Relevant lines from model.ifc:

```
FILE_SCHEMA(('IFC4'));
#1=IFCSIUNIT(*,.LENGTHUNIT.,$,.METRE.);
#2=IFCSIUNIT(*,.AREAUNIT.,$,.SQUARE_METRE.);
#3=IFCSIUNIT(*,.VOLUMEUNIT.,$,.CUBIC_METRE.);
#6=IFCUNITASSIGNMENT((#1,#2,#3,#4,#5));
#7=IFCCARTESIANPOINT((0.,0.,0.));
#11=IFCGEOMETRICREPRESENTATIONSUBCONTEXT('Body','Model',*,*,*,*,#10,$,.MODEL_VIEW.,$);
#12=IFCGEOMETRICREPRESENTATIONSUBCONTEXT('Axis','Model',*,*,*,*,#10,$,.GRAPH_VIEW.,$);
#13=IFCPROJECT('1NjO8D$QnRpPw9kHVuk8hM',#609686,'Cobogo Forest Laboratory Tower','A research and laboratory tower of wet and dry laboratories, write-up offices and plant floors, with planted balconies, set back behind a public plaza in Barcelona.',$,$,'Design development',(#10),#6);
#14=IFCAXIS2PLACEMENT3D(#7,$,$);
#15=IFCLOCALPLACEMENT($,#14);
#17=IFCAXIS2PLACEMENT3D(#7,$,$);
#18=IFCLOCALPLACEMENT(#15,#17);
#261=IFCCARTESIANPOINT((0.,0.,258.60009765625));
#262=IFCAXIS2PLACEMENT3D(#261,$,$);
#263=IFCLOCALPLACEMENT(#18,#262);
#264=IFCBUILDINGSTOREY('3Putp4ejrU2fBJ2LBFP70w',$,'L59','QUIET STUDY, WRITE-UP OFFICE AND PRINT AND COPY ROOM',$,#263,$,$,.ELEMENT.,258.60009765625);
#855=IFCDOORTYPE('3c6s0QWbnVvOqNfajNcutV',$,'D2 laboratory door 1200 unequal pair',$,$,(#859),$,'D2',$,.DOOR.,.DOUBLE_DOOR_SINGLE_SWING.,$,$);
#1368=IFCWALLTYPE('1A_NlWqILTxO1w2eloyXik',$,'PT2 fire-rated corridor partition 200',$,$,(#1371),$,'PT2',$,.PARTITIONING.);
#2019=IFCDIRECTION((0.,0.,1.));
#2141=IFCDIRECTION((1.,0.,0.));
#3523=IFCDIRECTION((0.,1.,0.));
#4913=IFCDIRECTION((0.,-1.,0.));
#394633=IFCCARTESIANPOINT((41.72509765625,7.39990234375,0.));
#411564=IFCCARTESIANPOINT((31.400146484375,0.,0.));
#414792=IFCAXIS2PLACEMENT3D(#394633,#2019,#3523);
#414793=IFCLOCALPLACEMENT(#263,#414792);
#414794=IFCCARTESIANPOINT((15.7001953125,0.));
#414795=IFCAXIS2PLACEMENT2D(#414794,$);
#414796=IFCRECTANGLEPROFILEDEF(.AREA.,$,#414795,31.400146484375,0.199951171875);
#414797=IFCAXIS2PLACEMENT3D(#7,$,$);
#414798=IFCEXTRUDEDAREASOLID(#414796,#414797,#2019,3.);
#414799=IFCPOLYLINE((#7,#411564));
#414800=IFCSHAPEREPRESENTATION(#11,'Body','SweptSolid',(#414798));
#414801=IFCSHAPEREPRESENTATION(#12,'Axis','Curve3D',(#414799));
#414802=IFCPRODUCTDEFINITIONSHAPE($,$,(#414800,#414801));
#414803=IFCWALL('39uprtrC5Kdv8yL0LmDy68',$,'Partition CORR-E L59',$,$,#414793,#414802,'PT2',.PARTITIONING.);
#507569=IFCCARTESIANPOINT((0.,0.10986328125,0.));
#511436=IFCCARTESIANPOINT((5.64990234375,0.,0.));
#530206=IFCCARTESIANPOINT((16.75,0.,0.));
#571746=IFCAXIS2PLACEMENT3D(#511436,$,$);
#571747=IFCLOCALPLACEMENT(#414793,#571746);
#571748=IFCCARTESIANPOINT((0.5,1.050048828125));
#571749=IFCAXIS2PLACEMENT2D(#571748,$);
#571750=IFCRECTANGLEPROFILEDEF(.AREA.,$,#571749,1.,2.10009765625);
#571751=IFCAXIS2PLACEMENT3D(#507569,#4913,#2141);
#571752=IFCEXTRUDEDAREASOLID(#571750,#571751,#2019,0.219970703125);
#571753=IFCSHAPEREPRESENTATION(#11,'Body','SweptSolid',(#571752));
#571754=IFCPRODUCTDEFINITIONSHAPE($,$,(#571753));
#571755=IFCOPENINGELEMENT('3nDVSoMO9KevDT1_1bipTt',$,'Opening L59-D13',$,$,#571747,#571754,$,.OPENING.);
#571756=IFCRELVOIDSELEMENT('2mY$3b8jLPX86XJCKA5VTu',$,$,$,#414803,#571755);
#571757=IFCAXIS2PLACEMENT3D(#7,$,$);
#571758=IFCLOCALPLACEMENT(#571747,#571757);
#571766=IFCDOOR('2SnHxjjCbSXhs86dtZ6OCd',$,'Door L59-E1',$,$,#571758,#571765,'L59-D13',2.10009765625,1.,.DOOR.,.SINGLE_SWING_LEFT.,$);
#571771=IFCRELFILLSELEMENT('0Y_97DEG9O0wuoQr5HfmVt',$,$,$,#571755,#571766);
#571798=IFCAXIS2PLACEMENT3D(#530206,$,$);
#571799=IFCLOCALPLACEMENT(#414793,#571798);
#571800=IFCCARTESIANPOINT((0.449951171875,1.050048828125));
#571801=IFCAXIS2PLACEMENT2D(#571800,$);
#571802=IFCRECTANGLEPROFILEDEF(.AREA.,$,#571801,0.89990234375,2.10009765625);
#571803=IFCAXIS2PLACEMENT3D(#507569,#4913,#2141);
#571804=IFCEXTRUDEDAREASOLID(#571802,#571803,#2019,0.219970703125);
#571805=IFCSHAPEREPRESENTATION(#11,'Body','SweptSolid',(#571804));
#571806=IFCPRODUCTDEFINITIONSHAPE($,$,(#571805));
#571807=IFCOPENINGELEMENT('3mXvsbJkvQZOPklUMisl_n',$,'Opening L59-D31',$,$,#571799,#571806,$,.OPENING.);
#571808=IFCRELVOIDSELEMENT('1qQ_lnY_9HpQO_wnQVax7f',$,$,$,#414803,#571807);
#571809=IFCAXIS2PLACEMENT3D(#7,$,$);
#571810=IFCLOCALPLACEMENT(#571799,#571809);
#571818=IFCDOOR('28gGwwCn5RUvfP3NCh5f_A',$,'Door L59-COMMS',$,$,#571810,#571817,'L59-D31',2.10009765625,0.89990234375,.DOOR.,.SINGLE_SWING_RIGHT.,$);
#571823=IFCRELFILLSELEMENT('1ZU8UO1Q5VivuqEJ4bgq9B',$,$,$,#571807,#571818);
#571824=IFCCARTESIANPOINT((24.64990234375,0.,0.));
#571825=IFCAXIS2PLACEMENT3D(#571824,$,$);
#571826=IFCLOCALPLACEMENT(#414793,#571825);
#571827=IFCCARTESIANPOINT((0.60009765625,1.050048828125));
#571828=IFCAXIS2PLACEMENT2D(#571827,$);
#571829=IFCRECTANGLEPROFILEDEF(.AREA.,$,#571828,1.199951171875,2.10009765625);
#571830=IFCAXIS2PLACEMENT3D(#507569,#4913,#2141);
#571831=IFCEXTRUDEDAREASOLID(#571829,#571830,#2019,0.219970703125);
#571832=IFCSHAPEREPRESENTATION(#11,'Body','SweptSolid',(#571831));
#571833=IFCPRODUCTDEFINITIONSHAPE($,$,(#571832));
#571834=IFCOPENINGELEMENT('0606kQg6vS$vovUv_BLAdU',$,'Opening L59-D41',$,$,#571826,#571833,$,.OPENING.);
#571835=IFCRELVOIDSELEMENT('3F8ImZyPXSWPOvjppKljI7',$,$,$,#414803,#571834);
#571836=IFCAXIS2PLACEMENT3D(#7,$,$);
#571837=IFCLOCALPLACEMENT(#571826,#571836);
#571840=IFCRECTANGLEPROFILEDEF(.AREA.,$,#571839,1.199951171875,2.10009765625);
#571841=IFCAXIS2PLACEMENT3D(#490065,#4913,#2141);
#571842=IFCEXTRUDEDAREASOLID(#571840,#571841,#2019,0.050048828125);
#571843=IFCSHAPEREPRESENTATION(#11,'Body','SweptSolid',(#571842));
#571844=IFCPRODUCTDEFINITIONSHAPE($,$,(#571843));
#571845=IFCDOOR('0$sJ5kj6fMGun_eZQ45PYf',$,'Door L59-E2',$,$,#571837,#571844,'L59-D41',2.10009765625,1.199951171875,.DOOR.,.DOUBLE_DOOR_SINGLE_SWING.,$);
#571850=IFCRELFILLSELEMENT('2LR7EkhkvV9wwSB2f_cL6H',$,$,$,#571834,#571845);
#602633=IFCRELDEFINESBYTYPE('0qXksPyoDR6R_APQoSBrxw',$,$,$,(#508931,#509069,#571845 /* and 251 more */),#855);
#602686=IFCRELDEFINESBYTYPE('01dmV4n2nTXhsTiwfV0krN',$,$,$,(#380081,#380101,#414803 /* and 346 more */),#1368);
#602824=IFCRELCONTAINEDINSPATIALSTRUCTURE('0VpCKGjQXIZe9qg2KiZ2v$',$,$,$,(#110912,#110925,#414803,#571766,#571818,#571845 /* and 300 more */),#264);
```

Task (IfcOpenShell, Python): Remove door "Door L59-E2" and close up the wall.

```python
import ifcopenshell
import ifcopenshell.api.feature
import ifcopenshell.api.root
import ifcopenshell.geom
import ifcopenshell.util.shape

model = ifcopenshell.open("model.ifc")
settings = ifcopenshell.geom.settings()


def volume(element):
    """Net volume in cubic metres, openings subtracted."""
    shape = ifcopenshell.geom.create_shape(settings, element)
    return ifcopenshell.util.shape.get_volume(shape.geometry)


door = model.by_guid("0$sJ5kj6fMGun_eZQ45PYf")
opening = door.FillsVoids[0].RelatingOpeningElement
wall = opening.VoidsElements[0].RelatingBuildingElement
before = volume(wall)

ifcopenshell.api.root.remove_product(model, product=door)
ifcopenshell.api.feature.remove_feature(model, feature=opening)

after = volume(wall)

print(f"wall volume {before:.3f} -> {after:.3f} m3")

model.write("model-out.ifc")
```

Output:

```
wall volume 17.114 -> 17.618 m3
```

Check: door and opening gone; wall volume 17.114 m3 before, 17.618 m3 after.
